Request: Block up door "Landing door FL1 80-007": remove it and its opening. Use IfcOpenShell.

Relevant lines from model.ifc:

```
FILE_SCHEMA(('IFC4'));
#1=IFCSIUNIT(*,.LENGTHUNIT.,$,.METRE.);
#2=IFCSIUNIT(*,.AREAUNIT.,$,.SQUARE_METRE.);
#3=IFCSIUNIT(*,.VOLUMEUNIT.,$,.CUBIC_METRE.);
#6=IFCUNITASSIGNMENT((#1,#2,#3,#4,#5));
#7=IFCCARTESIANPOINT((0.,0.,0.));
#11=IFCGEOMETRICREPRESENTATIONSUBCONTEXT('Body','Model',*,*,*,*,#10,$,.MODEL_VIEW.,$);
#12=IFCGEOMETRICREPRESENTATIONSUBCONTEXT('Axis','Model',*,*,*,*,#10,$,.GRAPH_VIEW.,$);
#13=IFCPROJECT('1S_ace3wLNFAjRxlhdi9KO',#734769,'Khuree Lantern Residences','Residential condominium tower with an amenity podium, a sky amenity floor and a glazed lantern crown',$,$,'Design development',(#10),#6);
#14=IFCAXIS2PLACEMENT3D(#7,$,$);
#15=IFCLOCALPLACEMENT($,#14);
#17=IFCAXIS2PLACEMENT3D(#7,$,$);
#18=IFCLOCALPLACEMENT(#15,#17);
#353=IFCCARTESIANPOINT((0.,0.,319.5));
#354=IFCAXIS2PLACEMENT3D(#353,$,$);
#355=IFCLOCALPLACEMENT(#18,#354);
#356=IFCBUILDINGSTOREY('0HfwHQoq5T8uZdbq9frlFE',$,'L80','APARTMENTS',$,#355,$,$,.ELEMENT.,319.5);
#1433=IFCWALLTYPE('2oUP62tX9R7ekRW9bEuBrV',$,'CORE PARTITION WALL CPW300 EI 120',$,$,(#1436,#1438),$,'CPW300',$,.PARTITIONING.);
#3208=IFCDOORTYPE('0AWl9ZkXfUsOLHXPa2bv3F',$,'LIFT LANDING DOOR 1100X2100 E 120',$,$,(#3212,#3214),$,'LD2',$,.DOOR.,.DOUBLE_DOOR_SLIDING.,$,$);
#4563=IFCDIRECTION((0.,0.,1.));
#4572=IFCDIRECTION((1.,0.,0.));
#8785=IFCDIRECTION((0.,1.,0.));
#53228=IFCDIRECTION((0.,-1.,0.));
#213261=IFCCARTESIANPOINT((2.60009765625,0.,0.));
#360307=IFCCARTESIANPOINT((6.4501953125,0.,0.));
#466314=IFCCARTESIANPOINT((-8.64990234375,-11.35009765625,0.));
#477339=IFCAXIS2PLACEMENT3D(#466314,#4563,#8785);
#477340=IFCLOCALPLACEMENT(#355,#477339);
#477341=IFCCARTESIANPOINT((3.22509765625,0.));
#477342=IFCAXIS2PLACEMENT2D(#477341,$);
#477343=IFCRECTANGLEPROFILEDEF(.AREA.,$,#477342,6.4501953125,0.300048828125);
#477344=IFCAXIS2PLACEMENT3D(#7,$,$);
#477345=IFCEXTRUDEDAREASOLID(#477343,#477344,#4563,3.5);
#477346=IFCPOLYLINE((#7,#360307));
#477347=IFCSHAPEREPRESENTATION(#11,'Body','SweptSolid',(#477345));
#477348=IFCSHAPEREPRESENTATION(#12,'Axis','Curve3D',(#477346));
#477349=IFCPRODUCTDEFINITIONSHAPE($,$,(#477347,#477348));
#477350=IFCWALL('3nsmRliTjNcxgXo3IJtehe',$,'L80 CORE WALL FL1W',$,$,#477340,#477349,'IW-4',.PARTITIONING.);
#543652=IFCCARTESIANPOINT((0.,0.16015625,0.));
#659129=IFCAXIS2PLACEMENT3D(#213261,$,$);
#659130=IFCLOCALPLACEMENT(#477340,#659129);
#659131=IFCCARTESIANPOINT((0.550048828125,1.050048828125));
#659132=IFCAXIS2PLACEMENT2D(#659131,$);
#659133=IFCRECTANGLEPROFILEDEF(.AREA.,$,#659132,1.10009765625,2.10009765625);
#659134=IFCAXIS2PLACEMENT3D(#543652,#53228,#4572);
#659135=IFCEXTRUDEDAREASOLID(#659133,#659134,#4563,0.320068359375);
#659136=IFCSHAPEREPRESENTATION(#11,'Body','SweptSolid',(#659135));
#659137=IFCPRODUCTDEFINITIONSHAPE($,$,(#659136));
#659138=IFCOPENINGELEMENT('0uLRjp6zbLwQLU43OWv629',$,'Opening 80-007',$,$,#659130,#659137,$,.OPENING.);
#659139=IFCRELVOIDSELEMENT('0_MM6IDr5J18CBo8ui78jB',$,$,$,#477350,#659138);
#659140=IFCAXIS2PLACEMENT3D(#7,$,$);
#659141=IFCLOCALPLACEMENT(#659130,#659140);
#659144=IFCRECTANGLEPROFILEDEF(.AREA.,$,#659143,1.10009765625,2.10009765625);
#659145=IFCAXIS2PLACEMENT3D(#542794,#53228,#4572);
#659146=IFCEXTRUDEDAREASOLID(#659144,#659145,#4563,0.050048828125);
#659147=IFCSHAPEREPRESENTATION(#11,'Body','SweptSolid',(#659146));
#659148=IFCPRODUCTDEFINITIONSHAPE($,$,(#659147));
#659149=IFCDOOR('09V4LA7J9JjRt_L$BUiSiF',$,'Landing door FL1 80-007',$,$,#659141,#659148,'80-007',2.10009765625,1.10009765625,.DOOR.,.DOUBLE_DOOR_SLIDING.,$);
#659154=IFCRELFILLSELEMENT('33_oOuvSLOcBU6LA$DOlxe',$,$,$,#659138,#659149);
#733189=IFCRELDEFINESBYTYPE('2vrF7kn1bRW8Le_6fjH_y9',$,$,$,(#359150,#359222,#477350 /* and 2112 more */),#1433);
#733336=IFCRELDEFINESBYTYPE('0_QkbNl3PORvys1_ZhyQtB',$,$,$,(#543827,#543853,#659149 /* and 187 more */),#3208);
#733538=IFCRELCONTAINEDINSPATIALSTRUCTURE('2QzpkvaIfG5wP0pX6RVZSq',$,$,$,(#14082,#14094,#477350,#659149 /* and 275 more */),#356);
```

```python
import ifcopenshell
import ifcopenshell.api.feature
import ifcopenshell.api.root
import ifcopenshell.geom
import ifcopenshell.util.shape

model = ifcopenshell.open("model.ifc")
settings = ifcopenshell.geom.settings()


def volume(element):
    """Net volume in cubic metres, openings subtracted."""
    shape = ifcopenshell.geom.create_shape(settings, element)
    return ifcopenshell.util.shape.get_volume(shape.geometry)


door = model.by_id(659149)
opening = door.FillsVoids[0].RelatingOpeningElement
wall = opening.VoidsElements[0].RelatingBuildingElement
before = volume(wall)

ifcopenshell.api.root.remove_product(model, product=door)
ifcopenshell.api.feature.remove_feature(model, feature=opening)

after = volume(wall)

print(f"wall volume {before:.3f} -> {after:.3f} m3")

model.write("model_v2.ifc")
```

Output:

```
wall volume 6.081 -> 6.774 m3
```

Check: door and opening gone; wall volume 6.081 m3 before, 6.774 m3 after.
